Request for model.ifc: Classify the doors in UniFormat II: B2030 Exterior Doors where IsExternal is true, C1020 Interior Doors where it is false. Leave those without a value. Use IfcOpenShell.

First a look at what the model holds.

```python
import ifcopenshell
import ifcopenshell.util.element

model = ifcopenshell.open("model.ifc")
print(model.schema)
print("classifications:", [c.Name for c in model.by_type("IfcClassification")])
values = [ifcopenshell.util.element.get_pset(e, "Pset_DoorCommon", "IsExternal") for e in model.by_type("IfcDoor")]
for value in (True, False, None):
    print("IsExternal", value, values.count(value))
```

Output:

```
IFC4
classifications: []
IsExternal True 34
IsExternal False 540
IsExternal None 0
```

```python
import ifcopenshell
import ifcopenshell.api.classification
import ifcopenshell.util.element

model = ifcopenshell.open("model.ifc")

system = ifcopenshell.api.classification.add_classification(model, classification="UniFormat II")

doors = model.by_type("IfcDoor")
external = {e: ifcopenshell.util.element.get_pset(e, "Pset_DoorCommon", "IsExternal") for e in doors}
for flag, code, name in ((True, "B2030", "Exterior Doors"), (False, "C1020", "Interior Doors")):
    products = [e for e in doors if external[e] is flag]
    ifcopenshell.api.classification.add_reference(
        model, products=products, classification=system, identification=code, name=name
    )
    print(code, len(products))

model.write("model_updated.ifc")
```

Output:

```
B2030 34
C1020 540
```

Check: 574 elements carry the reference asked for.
